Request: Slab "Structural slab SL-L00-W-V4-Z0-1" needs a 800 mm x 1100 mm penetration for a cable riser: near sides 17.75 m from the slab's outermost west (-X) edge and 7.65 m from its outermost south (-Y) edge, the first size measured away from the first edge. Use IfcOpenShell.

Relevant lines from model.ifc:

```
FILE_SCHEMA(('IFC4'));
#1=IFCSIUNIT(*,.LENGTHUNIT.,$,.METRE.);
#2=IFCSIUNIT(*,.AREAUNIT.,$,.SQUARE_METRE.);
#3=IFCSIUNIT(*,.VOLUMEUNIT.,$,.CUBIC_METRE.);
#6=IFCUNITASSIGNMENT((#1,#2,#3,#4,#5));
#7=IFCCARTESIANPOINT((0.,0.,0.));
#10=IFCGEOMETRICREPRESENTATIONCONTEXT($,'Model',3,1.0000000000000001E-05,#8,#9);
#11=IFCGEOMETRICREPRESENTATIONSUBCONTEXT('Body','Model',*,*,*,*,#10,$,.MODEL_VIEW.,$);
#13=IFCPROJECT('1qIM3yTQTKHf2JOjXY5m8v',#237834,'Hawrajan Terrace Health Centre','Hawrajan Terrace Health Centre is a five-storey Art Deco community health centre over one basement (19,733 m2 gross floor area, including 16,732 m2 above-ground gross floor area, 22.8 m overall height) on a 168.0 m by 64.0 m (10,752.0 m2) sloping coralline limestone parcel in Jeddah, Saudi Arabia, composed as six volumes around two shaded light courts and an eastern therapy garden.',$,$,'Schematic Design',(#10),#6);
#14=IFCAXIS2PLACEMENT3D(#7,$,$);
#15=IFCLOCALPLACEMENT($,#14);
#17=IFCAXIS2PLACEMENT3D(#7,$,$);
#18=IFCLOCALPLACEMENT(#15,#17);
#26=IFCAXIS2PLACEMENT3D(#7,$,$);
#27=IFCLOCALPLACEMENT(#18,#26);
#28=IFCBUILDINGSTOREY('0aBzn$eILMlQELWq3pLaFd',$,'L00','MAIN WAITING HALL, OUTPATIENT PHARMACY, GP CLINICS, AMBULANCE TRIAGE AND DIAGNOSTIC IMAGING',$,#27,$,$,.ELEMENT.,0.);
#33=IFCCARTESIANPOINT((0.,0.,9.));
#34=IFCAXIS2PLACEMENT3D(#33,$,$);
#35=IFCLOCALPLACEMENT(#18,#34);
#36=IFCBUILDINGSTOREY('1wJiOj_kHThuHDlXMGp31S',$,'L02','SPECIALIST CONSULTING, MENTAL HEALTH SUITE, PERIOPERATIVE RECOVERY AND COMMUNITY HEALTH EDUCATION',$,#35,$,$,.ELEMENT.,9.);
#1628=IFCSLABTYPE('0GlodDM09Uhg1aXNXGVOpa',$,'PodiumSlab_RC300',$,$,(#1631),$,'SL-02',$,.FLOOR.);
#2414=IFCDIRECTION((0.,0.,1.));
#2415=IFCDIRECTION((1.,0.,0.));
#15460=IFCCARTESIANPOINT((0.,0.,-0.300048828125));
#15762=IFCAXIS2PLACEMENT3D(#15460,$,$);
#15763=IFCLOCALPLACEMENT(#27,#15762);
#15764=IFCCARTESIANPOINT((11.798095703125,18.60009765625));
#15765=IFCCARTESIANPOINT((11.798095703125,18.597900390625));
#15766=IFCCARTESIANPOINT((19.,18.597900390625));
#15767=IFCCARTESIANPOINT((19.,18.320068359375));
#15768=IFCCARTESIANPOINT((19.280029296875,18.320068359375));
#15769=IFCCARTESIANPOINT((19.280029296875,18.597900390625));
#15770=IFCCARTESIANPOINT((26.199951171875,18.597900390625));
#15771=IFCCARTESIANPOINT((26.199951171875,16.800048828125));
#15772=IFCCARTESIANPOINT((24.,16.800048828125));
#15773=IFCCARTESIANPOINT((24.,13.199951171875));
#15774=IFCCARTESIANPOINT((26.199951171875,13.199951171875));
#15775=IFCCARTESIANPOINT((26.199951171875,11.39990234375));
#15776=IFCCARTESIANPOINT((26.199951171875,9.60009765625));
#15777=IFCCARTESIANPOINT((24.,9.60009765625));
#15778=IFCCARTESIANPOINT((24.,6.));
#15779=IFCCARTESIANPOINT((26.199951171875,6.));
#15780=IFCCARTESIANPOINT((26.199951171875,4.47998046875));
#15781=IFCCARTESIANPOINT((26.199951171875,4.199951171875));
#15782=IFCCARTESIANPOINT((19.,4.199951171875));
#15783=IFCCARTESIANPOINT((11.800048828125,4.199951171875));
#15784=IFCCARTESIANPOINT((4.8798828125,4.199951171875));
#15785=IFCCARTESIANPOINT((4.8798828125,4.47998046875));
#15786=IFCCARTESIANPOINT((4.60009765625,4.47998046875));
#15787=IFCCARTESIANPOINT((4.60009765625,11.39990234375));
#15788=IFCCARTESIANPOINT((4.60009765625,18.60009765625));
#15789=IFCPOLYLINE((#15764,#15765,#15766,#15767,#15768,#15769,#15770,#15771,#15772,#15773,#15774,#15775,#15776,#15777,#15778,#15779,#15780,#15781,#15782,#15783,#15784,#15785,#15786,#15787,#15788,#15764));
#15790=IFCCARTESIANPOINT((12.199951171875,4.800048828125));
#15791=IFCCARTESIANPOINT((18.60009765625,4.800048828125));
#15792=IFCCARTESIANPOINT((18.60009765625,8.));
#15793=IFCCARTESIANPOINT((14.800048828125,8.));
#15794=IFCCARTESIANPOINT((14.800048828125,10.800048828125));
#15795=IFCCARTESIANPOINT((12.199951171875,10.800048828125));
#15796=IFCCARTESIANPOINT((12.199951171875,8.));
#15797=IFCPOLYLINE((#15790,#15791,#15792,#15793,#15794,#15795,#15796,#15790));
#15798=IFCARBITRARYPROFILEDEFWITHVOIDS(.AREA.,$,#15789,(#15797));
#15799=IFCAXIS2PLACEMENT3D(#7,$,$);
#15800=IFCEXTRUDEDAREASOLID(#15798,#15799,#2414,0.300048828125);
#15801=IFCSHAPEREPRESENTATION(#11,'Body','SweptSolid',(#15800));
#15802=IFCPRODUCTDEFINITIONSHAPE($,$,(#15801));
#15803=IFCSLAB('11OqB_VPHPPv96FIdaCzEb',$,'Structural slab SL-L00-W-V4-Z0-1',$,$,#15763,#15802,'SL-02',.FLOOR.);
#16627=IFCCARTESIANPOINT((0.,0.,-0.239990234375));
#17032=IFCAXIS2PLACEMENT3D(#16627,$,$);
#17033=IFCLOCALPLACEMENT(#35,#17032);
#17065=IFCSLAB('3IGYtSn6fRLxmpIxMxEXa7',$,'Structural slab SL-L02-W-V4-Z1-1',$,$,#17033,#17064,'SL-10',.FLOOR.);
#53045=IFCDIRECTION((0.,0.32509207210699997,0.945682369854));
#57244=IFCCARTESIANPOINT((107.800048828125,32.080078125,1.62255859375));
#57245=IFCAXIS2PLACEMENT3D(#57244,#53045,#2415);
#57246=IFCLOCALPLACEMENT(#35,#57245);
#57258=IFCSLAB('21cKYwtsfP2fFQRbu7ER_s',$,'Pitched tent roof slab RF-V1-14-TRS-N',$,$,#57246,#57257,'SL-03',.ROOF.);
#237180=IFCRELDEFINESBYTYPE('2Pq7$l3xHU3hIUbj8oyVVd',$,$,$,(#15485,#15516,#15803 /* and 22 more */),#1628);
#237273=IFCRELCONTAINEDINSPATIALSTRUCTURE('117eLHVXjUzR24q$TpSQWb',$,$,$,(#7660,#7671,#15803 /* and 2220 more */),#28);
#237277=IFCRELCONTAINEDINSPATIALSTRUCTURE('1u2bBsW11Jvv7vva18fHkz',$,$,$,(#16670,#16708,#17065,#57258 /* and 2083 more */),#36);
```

```python
import numpy as np
import ifcopenshell
import ifcopenshell.api.feature
import ifcopenshell.api.geometry
import ifcopenshell.api.root
import ifcopenshell.geom
import ifcopenshell.util.placement
import ifcopenshell.util.representation
import ifcopenshell.util.shape
import ifcopenshell.util.unit

model = ifcopenshell.open("model.ifc")
unit_scale = ifcopenshell.util.unit.calculate_unit_scale(model)
settings = ifcopenshell.geom.settings()


def volume(element):
    """Net volume in cubic metres, openings subtracted."""
    shape = ifcopenshell.geom.create_shape(settings, element)
    return ifcopenshell.util.shape.get_volume(shape.geometry)


slab = model.by_guid("11OqB_VPHPPv96FIdaCzEb")
before = volume(slab)

# Extent in the slab's own axes, in metres. The edges named are its -X and -Y sides.
slab_shape = ifcopenshell.geom.create_shape(settings, slab)
vertices = ifcopenshell.util.shape.get_vertices(slab_shape.geometry)
x_min, y_min, bottom = vertices.min(axis=0)
top = vertices[:, 2].max()

opening = ifcopenshell.api.root.create_entity(model, ifc_class="IfcOpeningElement", name="Cable riser opening", predefined_type="OPENING")
context = ifcopenshell.util.representation.get_context(model, "Model", "Body", "MODEL_VIEW")
width, depth = 0.8, 1.1
outline = [(0.0, 0.0), (width, 0.0), (width, depth), (0.0, depth), (0.0, 0.0)]
# Overshoot both faces by 50 mm so the cut is clean.
shape = ifcopenshell.api.geometry.add_slab_representation(
    model, context=context, depth=top - bottom + 0.1, polyline=outline
)
ifcopenshell.api.geometry.assign_representation(model, product=opening, representation=shape)

matrix = ifcopenshell.util.placement.get_local_placement(slab.ObjectPlacement)
matrix[:, 3] = matrix @ np.append(np.array([x_min + 17.75, y_min + 7.65, bottom - 0.05]) / unit_scale, 1.0)
ifcopenshell.api.geometry.edit_object_placement(model, product=opening, matrix=matrix, is_si=False)
ifcopenshell.api.feature.add_feature(model, feature=opening, element=slab)

after = volume(slab)

print(f"slab volume {before:.3f} -> {after:.3f} m3")

model.write("model-out.ifc")
```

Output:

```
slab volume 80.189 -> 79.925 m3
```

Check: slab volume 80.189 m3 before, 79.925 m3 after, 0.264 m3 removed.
